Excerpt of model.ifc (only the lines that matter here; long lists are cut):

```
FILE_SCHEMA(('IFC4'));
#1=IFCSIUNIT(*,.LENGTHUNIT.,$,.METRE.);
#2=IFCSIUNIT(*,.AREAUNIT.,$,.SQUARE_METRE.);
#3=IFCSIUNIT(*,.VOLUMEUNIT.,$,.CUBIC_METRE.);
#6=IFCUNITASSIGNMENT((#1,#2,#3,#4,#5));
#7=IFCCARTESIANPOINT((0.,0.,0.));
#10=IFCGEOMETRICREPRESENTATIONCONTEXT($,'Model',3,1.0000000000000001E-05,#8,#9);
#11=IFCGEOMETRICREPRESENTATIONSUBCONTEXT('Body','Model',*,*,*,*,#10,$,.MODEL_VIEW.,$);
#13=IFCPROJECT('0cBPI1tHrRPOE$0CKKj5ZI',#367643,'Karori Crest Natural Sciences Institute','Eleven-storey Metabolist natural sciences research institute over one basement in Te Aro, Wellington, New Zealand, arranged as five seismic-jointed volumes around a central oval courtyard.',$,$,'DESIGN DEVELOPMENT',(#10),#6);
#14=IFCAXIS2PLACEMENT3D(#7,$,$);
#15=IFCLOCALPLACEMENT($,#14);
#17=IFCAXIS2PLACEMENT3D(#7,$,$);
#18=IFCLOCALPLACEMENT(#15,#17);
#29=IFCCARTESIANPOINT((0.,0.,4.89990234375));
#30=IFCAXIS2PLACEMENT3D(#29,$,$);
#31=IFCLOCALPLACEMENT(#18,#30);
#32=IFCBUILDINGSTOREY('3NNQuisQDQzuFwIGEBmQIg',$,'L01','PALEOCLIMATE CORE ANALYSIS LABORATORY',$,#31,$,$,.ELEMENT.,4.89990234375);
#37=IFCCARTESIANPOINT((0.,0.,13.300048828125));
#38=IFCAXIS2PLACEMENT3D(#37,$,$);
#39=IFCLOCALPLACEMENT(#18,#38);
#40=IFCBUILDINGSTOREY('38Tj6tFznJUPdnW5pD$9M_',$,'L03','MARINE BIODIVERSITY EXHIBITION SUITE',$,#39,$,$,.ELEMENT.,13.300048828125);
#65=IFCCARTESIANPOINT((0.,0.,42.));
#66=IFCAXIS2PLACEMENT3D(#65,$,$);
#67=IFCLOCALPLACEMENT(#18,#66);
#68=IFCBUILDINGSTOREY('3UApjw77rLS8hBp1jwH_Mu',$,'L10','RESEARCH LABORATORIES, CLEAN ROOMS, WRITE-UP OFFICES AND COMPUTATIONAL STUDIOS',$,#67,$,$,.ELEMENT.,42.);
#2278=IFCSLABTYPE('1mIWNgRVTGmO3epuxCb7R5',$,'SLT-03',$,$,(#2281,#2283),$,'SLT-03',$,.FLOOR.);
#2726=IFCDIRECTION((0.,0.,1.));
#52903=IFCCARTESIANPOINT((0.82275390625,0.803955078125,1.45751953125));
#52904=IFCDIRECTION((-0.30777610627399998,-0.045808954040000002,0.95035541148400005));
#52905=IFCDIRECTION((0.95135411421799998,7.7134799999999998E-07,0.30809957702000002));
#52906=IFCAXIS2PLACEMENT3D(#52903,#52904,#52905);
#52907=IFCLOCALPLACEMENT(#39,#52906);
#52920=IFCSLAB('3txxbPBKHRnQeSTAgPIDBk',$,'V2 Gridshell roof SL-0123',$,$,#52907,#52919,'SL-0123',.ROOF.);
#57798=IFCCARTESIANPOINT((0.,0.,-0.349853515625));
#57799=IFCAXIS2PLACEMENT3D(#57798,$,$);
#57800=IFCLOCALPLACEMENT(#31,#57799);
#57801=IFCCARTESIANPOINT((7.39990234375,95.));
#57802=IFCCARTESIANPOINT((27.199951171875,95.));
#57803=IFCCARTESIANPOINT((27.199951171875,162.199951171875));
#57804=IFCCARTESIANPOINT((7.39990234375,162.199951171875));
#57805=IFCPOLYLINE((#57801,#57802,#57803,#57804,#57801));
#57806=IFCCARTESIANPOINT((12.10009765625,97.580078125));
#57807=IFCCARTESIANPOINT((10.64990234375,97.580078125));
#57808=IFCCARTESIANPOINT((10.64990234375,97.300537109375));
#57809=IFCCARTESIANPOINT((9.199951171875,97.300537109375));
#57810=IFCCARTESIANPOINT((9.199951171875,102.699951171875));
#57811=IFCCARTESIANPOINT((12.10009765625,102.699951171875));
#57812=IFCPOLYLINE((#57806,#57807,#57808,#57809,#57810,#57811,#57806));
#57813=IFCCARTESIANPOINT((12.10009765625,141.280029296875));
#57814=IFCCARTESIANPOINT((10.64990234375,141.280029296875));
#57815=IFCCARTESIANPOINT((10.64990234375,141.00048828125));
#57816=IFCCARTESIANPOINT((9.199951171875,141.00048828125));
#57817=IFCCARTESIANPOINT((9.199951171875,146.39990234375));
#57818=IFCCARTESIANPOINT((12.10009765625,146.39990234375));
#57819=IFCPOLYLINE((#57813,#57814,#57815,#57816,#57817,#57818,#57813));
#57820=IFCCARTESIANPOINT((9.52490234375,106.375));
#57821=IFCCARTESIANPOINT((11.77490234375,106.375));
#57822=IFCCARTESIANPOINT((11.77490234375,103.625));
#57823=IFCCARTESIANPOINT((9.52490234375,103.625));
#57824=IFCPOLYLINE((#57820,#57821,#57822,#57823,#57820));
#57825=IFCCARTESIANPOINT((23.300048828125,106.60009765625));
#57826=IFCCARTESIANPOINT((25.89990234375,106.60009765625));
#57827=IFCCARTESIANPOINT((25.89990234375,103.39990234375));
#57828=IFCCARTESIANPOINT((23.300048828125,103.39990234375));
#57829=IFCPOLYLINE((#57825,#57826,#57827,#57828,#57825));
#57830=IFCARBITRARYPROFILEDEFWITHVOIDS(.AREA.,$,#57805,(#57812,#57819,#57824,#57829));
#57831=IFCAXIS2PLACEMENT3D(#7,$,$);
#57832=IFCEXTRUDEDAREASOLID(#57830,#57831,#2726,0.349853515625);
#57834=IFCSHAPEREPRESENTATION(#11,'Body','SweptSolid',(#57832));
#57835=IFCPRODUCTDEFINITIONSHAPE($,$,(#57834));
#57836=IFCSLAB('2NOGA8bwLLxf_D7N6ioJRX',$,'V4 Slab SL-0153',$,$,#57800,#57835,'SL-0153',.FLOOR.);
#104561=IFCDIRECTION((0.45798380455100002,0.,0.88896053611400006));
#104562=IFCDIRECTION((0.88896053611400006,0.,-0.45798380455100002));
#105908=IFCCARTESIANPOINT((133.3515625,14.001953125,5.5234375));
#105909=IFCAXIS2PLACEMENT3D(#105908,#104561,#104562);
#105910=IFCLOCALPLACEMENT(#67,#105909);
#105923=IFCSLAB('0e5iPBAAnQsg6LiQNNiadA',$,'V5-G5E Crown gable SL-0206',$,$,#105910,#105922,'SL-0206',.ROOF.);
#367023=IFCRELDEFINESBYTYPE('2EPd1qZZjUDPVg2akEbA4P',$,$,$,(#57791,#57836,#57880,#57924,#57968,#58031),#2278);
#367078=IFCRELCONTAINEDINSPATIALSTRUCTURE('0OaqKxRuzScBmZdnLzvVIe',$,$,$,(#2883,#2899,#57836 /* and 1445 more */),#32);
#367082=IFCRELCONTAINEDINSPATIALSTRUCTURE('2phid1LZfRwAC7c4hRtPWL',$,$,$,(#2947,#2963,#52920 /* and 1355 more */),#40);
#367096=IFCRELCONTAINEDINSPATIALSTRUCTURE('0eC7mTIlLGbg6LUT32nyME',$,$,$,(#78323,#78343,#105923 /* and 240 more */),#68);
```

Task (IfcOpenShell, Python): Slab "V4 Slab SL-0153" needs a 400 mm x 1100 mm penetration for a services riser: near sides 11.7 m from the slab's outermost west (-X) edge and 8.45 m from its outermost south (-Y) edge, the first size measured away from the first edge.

```python
import numpy as np
import ifcopenshell
import ifcopenshell.api.feature
import ifcopenshell.api.geometry
import ifcopenshell.api.root
import ifcopenshell.geom
import ifcopenshell.util.placement
import ifcopenshell.util.representation
import ifcopenshell.util.shape
import ifcopenshell.util.unit

model = ifcopenshell.open("model.ifc")
unit_scale = ifcopenshell.util.unit.calculate_unit_scale(model)
settings = ifcopenshell.geom.settings()


def volume(element):
    """Net volume in cubic metres, openings subtracted."""
    shape = ifcopenshell.geom.create_shape(settings, element)
    return ifcopenshell.util.shape.get_volume(shape.geometry)


slab = model.by_guid("2NOGA8bwLLxf_D7N6ioJRX")
before = volume(slab)

# Extent in the slab's own axes, in metres. The edges named are its -X and -Y sides.
slab_shape = ifcopenshell.geom.create_shape(settings, slab)
vertices = ifcopenshell.util.shape.get_vertices(slab_shape.geometry)
x_min, y_min, bottom = vertices.min(axis=0)
top = vertices[:, 2].max()

opening = ifcopenshell.api.root.create_entity(model, ifc_class="IfcOpeningElement", name="Services riser opening", predefined_type="OPENING")
context = ifcopenshell.util.representation.get_context(model, "Model", "Body", "MODEL_VIEW")
width, depth = 0.4, 1.1
outline = [(0.0, 0.0), (width, 0.0), (width, depth), (0.0, depth), (0.0, 0.0)]
# Overshoot both faces by 50 mm so the cut is clean.
shape = ifcopenshell.api.geometry.add_slab_representation(
    model, context=context, depth=top - bottom + 0.1, polyline=outline
)
ifcopenshell.api.geometry.assign_representation(model, product=opening, representation=shape)

matrix = ifcopenshell.util.placement.get_local_placement(slab.ObjectPlacement)
matrix[:, 3] = matrix @ np.append(np.array([x_min + 11.7, y_min + 8.45, bottom - 0.05]) / unit_scale, 1.0)
ifcopenshell.api.geometry.edit_object_placement(model, product=opening, matrix=matrix, is_si=False)
ifcopenshell.api.feature.add_feature(model, feature=opening, element=slab)

after = volume(slab)

print(f"slab volume {before:.3f} -> {after:.3f} m3")

model.write("model-out.ifc")
```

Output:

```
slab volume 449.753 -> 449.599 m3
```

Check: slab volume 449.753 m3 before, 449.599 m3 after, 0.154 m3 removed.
